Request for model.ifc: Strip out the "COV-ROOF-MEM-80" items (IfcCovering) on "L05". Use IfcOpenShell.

First a look at what the model holds.

```python
import ifcopenshell
import ifcopenshell.util.element

model = ifcopenshell.open("model.ifc")
print(model.schema)
storey = next(s for s in model.by_type("IfcBuildingStorey") if s.Name == "L05")
coverings = [e for e in ifcopenshell.util.element.get_decomposition(storey) if e.is_a("IfcCovering")]
seen = {}
for e in coverings:
    element_type = ifcopenshell.util.element.get_type(e)
    name = element_type.Name if element_type not in (None, e) else None
    seen[name] = seen.get(name, 0) + 1
for name, count in sorted(seen.items(), key=str):
    print(count, "x", name)
```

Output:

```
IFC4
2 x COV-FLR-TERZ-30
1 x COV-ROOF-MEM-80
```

```python
import ifcopenshell
import ifcopenshell.api.root
import ifcopenshell.util.element

model = ifcopenshell.open("model.ifc")

storey = next(s for s in model.by_type("IfcBuildingStorey") if s.Name == "L05")
coverings = [e for e in ifcopenshell.util.element.get_decomposition(storey) if e.is_a("IfcCovering")]
targets = [e for e in coverings if (t := ifcopenshell.util.element.get_type(e)) not in (None, e) and t.Name == "COV-ROOF-MEM-80"]

for e in targets:
    ifcopenshell.api.root.remove_product(model, product=e)
print(len(targets), "removed")

model.write("model-out.ifc")
```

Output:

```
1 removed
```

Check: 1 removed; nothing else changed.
